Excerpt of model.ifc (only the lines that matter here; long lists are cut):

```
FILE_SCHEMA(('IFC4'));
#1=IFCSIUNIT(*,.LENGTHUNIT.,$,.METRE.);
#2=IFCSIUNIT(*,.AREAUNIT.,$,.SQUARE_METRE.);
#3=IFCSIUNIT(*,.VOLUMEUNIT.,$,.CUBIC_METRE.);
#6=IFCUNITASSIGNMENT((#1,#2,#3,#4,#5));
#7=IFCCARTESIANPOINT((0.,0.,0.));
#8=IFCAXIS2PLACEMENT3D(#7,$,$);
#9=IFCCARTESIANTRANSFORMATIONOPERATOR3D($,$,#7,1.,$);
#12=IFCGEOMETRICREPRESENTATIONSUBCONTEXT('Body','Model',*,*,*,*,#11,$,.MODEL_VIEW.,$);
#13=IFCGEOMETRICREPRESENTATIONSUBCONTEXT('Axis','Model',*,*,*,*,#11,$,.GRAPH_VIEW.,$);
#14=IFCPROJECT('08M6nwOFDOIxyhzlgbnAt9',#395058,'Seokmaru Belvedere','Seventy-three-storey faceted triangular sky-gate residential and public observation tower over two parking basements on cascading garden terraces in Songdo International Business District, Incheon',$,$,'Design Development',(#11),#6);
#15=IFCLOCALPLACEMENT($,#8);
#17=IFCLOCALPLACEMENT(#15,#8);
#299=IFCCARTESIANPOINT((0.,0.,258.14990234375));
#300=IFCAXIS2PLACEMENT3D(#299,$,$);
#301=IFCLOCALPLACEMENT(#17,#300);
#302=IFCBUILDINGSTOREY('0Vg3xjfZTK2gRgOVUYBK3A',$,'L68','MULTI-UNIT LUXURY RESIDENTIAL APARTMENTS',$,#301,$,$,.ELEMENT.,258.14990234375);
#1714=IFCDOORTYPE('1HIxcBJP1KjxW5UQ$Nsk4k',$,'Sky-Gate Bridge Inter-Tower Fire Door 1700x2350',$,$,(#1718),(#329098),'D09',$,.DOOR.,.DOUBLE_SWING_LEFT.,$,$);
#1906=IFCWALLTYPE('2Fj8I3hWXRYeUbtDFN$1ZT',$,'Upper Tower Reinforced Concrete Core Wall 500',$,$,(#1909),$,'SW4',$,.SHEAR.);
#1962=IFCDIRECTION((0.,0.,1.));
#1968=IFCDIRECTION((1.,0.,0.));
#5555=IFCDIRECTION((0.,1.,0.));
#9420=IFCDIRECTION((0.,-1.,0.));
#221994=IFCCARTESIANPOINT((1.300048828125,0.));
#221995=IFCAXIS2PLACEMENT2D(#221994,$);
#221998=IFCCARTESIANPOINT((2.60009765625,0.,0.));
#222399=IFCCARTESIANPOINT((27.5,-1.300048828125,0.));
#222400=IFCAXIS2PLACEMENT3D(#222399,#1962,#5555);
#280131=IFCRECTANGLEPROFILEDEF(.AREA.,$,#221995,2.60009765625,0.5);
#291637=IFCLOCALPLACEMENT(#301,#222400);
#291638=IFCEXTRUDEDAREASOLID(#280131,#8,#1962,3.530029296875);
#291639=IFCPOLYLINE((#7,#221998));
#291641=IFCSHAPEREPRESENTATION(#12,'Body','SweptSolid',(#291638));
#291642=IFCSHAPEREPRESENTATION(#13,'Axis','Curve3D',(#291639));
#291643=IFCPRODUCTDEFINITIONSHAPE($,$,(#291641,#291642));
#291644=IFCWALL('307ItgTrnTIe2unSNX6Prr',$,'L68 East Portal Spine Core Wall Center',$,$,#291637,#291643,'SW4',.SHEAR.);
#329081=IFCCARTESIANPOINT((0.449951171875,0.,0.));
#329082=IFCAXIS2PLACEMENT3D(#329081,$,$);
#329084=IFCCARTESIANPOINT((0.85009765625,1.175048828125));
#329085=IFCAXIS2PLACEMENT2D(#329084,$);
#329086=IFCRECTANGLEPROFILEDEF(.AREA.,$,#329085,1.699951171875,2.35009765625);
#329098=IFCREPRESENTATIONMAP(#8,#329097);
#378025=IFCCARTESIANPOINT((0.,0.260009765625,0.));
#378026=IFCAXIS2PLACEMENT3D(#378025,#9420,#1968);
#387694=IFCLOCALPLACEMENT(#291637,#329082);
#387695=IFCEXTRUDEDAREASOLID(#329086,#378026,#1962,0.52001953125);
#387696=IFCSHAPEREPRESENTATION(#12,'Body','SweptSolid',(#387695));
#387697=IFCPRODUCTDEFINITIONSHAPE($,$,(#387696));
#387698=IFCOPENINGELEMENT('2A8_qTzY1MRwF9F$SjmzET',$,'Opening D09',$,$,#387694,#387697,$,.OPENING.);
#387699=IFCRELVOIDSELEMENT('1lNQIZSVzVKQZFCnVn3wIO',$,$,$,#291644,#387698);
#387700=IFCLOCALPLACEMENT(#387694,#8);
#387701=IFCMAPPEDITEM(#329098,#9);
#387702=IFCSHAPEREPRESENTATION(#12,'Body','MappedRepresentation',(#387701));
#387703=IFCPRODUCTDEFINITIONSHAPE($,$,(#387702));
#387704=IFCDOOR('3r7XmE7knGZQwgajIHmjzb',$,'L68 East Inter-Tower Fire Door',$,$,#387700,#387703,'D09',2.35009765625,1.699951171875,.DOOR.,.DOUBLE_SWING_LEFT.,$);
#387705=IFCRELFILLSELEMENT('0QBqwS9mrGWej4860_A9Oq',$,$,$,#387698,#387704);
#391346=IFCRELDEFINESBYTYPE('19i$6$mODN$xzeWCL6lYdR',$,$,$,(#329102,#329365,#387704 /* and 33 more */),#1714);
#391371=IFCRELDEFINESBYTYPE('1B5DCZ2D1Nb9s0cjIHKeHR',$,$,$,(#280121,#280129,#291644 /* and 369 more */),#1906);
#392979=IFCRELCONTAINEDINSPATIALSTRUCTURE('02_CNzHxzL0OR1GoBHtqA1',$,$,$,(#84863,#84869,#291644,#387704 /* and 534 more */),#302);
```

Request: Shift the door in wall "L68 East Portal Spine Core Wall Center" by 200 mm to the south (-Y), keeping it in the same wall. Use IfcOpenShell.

```python
import ifcopenshell
import ifcopenshell.api.geometry
import ifcopenshell.util.placement
import ifcopenshell.util.unit

model = ifcopenshell.open("model.ifc")
unit_scale = ifcopenshell.util.unit.calculate_unit_scale(model)

door = model.by_guid("3r7XmE7knGZQwgajIHmjzb")
opening = door.FillsVoids[0].RelatingOpeningElement
wall = opening.VoidsElements[0].RelatingBuildingElement

wall_matrix = ifcopenshell.util.placement.get_local_placement(wall.ObjectPlacement)
shift = wall_matrix[:3, 0] * -0.2 / unit_scale
before = ifcopenshell.util.placement.get_local_placement(door.ObjectPlacement)[:3, 3].copy()

# The door is placed relative to its opening, so it follows when the opening moves.
matrix = ifcopenshell.util.placement.get_local_placement(opening.ObjectPlacement)
matrix[:3, 3] += shift
ifcopenshell.api.geometry.edit_object_placement(
    model, product=opening, matrix=matrix, is_si=False, should_transform_children=True
)

after = ifcopenshell.util.placement.get_local_placement(door.ObjectPlacement)[:3, 3]
print("door moved by", (after - before).round(3) + 0.0)

model.write("model-out.ifc")
```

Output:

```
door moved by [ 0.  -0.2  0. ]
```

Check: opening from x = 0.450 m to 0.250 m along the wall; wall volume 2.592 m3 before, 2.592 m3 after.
